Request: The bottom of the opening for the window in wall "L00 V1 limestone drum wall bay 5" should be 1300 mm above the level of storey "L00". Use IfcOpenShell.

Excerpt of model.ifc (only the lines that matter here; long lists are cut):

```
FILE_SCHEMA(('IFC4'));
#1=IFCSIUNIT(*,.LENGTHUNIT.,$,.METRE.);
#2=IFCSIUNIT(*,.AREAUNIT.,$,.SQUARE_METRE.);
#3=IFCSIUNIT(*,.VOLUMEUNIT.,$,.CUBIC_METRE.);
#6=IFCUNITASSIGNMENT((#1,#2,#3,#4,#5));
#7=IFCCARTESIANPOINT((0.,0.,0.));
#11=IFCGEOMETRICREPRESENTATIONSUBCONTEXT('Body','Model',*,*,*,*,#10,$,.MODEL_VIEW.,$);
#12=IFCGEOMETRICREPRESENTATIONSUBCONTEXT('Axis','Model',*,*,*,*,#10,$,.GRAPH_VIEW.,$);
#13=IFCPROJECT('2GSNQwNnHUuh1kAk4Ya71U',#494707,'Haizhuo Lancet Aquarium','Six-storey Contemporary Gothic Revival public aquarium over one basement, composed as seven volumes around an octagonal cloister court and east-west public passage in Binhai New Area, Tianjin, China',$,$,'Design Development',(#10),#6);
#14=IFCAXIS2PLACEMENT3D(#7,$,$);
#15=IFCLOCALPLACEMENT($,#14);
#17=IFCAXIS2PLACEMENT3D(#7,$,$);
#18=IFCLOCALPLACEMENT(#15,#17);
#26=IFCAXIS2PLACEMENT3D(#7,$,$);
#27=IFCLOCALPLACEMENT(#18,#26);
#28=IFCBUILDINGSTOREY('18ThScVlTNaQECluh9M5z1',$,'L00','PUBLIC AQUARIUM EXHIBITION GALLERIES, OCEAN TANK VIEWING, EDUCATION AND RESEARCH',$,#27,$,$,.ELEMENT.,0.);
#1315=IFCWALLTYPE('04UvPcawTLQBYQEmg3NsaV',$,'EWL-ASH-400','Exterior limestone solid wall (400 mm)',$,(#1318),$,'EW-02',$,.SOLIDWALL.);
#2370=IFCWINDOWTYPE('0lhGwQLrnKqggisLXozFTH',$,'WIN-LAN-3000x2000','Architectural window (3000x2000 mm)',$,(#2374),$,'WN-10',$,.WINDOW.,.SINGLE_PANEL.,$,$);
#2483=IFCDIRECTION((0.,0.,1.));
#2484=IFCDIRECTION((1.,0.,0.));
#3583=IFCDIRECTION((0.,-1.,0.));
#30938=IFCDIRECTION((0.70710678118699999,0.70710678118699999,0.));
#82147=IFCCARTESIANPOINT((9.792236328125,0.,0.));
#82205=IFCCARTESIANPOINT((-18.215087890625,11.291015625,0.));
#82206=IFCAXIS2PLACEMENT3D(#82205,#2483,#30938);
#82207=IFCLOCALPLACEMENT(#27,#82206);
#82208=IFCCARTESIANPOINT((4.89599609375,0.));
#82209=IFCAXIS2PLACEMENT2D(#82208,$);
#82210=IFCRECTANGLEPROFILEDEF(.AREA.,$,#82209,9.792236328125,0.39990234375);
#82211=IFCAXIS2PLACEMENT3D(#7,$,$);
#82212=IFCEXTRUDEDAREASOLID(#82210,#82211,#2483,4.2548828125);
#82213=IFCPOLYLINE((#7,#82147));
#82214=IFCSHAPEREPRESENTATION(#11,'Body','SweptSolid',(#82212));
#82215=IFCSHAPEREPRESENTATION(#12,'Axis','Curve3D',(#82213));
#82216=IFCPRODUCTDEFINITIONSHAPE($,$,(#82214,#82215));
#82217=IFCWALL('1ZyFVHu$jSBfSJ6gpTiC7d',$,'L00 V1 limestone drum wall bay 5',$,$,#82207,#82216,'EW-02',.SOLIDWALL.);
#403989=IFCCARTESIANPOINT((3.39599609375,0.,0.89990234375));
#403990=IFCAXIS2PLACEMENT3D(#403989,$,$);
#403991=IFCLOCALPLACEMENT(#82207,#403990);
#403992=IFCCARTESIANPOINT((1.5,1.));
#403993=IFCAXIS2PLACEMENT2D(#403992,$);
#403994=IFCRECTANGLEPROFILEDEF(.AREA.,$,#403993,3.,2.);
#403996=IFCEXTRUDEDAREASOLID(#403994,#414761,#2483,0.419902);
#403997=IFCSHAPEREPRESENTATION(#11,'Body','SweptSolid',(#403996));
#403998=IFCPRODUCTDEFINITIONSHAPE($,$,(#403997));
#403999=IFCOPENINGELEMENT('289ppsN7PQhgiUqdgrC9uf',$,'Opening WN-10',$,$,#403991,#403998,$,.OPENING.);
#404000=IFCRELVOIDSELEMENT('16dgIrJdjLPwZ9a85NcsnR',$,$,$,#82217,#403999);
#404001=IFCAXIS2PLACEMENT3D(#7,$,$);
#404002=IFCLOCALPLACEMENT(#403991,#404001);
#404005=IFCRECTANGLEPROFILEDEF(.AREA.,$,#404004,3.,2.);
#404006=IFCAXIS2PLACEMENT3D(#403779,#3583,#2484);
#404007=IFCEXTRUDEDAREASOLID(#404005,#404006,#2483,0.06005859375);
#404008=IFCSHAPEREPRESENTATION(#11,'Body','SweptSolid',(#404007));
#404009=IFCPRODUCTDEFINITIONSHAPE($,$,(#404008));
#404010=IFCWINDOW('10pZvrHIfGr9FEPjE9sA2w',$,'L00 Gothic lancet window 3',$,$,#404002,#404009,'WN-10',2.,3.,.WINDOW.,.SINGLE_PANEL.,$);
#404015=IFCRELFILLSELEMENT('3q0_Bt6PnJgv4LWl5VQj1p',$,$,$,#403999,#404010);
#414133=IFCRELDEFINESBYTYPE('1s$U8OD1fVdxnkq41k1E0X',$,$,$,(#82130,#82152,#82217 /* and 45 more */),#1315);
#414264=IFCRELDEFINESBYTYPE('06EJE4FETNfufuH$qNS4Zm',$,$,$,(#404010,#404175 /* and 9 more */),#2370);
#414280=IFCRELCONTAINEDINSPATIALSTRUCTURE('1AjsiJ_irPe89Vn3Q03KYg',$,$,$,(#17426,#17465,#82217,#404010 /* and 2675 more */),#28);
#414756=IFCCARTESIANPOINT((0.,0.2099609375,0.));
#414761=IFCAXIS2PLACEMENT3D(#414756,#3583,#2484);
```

```python
import numpy as np
import ifcopenshell
import ifcopenshell.api.geometry
import ifcopenshell.geom
import ifcopenshell.util.element
import ifcopenshell.util.placement
import ifcopenshell.util.shape
import ifcopenshell.util.unit

model = ifcopenshell.open("model.ifc")
unit_scale = ifcopenshell.util.unit.calculate_unit_scale(model)

window = model.by_id(404010)
opening = window.FillsVoids[0].RelatingOpeningElement
storey = ifcopenshell.util.element.get_container(window, ifc_class="IfcBuildingStorey")
level = ifcopenshell.util.placement.get_local_placement(storey.ObjectPlacement)[2, 3]

# The opening's origin need not be at the sill, so measure its lowest point.
shape = ifcopenshell.geom.create_shape(ifcopenshell.geom.settings(), opening)
bottom = ifcopenshell.util.shape.get_shape_bottom_elevation(shape, shape.geometry) / unit_scale
dz = level + 1.3 - bottom

shift = np.array([0.0, 0.0, dz])
# The window is placed relative to its opening, so it follows when the opening moves.
matrix = ifcopenshell.util.placement.get_local_placement(opening.ObjectPlacement)
matrix[:3, 3] += shift
ifcopenshell.api.geometry.edit_object_placement(
    model, product=opening, matrix=matrix, is_si=False, should_transform_children=True
)

print(f"moved by {dz * unit_scale:+.3f} m")

model.write("model_v2.ifc")
```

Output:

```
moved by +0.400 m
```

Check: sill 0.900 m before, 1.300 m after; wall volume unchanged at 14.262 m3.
